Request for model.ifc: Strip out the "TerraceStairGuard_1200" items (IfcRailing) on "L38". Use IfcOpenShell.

First a look at what the model holds.

```python
import ifcopenshell
import ifcopenshell.util.element

model = ifcopenshell.open("model.ifc")
print(model.schema)
storey = next(s for s in model.by_type("IfcBuildingStorey") if s.Name == "L38")
railings = [e for e in ifcopenshell.util.element.get_decomposition(storey) if e.is_a("IfcRailing")]
seen = {}
for e in railings:
    element_type = ifcopenshell.util.element.get_type(e)
    name = element_type.Name if element_type not in (None, e) else None
    seen[name] = seen.get(name, 0) + 1
for name, count in sorted(seen.items(), key=str):
    print(count, "x", name)
```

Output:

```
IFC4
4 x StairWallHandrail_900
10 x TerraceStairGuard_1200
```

```python
import ifcopenshell
import ifcopenshell.api.root
import ifcopenshell.util.element

model = ifcopenshell.open("model.ifc")

storey = next(s for s in model.by_type("IfcBuildingStorey") if s.Name == "L38")
railings = [e for e in ifcopenshell.util.element.get_decomposition(storey) if e.is_a("IfcRailing")]
targets = [e for e in railings if (t := ifcopenshell.util.element.get_type(e)) not in (None, e) and t.Name == "TerraceStairGuard_1200"]

for e in targets:
    ifcopenshell.api.root.remove_product(model, product=e)
print(len(targets), "removed")

model.write("model-out.ifc")
```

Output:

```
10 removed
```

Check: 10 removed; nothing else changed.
